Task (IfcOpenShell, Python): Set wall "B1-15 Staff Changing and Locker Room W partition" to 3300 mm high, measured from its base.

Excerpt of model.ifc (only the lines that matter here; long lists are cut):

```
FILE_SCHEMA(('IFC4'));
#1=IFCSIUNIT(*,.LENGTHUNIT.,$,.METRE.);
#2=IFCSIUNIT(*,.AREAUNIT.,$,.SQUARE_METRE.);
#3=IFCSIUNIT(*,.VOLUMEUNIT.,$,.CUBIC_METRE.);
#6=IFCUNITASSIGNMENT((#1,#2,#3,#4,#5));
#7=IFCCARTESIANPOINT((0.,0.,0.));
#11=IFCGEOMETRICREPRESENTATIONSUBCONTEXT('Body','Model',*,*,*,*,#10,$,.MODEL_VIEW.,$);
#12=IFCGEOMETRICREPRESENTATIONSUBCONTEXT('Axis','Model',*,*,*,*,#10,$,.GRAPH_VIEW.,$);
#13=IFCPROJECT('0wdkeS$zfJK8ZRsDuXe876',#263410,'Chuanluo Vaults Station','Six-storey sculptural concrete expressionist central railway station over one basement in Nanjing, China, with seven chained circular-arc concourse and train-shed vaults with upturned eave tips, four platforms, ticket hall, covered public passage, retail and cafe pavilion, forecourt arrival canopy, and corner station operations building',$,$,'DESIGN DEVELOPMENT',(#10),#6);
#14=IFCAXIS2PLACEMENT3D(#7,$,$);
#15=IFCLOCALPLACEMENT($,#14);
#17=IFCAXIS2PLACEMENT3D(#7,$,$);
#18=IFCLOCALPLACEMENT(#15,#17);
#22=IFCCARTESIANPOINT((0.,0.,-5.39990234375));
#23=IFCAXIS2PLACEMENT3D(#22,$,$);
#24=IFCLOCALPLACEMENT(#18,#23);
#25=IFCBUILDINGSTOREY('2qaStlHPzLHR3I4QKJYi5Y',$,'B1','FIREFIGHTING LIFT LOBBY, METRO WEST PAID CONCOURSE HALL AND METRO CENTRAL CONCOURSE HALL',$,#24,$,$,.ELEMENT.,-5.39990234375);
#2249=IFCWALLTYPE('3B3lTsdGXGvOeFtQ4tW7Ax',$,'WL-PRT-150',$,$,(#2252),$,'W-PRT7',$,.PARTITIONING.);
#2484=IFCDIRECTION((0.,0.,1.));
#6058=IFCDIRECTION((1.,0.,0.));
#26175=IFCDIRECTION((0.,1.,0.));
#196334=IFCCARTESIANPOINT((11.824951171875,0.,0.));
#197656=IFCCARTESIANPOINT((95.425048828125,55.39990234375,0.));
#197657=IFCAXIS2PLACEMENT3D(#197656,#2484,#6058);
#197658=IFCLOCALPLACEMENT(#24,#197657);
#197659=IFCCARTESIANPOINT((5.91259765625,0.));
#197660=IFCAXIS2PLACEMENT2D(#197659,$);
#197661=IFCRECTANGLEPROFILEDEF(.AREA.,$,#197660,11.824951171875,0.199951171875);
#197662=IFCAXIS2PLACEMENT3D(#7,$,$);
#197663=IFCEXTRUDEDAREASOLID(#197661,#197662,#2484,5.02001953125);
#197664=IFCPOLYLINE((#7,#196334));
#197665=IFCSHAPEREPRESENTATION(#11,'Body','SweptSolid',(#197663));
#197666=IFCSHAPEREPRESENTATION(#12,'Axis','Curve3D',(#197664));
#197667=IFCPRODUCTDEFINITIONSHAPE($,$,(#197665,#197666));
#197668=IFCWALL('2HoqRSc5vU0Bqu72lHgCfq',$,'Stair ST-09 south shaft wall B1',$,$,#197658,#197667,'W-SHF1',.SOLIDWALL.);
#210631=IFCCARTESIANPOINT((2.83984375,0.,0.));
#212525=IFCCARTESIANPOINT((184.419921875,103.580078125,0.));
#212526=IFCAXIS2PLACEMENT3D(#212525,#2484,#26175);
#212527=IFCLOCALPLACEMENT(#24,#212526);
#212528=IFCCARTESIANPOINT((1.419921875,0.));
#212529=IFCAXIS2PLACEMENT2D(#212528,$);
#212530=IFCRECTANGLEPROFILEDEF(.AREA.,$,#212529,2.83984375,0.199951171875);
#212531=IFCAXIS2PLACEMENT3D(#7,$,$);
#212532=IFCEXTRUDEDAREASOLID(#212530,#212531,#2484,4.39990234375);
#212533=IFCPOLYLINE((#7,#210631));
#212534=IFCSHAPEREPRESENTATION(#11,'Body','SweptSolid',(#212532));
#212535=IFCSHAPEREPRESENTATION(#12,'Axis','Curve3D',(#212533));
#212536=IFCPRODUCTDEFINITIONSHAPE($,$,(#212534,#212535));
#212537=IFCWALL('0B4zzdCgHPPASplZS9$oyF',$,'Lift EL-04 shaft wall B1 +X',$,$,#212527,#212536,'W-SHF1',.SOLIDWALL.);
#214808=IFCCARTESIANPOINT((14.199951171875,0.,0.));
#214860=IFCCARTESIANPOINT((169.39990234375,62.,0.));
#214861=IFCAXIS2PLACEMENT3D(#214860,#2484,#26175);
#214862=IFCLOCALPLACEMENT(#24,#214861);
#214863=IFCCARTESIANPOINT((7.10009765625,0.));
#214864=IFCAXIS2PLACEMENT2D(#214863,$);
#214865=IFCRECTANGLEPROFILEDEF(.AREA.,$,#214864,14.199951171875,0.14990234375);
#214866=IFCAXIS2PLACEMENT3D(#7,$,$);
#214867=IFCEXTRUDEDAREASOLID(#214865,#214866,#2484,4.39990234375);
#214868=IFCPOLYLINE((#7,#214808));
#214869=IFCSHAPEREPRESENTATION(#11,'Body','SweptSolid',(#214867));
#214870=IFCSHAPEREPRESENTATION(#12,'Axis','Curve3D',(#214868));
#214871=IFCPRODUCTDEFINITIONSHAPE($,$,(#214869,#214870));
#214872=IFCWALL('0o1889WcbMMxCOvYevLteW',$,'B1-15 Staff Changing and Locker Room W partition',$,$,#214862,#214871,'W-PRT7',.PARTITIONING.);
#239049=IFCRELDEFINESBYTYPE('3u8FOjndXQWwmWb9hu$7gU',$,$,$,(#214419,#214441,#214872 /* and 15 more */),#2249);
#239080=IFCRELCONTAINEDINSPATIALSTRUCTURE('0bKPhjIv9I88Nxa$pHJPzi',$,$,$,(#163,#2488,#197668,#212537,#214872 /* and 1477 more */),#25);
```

```python
import ifcopenshell
import ifcopenshell.geom
import ifcopenshell.util.representation
import ifcopenshell.util.shape

model = ifcopenshell.open("model.ifc")
settings = ifcopenshell.geom.settings()


def volume(element):
    """Net volume in cubic metres, openings subtracted."""
    shape = ifcopenshell.geom.create_shape(settings, element)
    return ifcopenshell.util.shape.get_volume(shape.geometry)


wall = model.by_id(214872)
before = volume(wall)

body = ifcopenshell.util.representation.get_representation(wall, "Model", "Body")
solid = body.Items[0]
old_height = solid.Depth
solid.Depth = 3.3
after = volume(wall)

print(f"height {old_height:g} -> {solid.Depth:g}, volume {before:.3f} -> {after:.3f} m3")

model.write("model-out.ifc")
```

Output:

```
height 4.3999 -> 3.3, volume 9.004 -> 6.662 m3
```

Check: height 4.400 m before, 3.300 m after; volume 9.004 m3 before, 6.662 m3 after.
